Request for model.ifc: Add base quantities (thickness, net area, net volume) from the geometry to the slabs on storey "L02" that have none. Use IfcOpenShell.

First a look at what the model holds.

```python
import ifcopenshell
import ifcopenshell.util.element
import ifcopenshell.util.unit

model = ifcopenshell.open("model.ifc")
print(model.schema)
for unit_type in ("LENGTHUNIT", "AREAUNIT", "VOLUMEUNIT"):
    print(unit_type, ifcopenshell.util.unit.calculate_unit_scale(model, unit_type))
storey = next(s for s in model.by_type("IfcBuildingStorey") if s.Name == "L02")
slabs = [e for e in ifcopenshell.util.element.get_decomposition(storey) if e.is_a("IfcSlab")]
for e in sorted(slabs, key=lambda e: e.id()):
    print(e.id(), e.is_a(), e.Name, list(ifcopenshell.util.element.get_psets(e, qtos_only=True)), sep=" | ")
```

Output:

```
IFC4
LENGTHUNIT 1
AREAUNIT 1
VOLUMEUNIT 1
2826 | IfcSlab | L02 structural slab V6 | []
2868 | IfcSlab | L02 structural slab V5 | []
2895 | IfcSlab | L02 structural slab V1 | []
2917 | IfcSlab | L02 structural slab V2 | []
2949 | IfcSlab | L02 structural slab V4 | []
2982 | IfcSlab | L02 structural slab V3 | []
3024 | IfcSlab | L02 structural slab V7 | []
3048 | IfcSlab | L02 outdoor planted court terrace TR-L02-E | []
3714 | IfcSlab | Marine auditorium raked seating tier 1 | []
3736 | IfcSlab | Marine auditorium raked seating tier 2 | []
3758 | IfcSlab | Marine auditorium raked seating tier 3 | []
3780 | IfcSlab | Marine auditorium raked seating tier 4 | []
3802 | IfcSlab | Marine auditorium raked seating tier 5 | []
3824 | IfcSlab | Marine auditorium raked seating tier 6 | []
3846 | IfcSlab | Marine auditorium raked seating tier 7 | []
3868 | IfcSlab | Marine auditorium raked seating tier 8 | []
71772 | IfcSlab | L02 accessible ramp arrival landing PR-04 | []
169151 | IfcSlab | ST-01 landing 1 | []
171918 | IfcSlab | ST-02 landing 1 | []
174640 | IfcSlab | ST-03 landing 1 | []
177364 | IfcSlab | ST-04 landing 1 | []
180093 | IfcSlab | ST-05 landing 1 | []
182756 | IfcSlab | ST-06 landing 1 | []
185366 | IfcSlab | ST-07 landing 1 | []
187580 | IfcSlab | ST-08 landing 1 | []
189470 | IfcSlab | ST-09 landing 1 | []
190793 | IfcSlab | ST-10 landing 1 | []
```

```python
import ifcopenshell
import ifcopenshell.api.pset
import ifcopenshell.geom
import ifcopenshell.util.element
import ifcopenshell.util.shape
import ifcopenshell.util.unit

model = ifcopenshell.open("model.ifc")
unit_scale = ifcopenshell.util.unit.calculate_unit_scale(model)
area_scale = ifcopenshell.util.unit.calculate_unit_scale(model, "AREAUNIT")
volume_scale = ifcopenshell.util.unit.calculate_unit_scale(model, "VOLUMEUNIT")
settings = ifcopenshell.geom.settings()

storey = next(s for s in model.by_type("IfcBuildingStorey") if s.Name == "L02")
slabs = [e for e in ifcopenshell.util.element.get_decomposition(storey) if e.is_a("IfcSlab")]

for e in sorted(slabs, key=lambda e: e.id()):
    if ifcopenshell.util.element.get_psets(e, qtos_only=True, should_inherit=False):
        continue
    # Geometry comes back in metres, in the element's own axes.
    shape = ifcopenshell.geom.create_shape(settings, e)
    values = {
        "Width": ifcopenshell.util.shape.get_z(shape.geometry) / unit_scale,
        "NetArea": ifcopenshell.util.shape.get_footprint_area(shape.geometry) / area_scale,
        "NetVolume": ifcopenshell.util.shape.get_volume(shape.geometry) / volume_scale,
    }
    qto = ifcopenshell.api.pset.add_qto(model, product=e, name="Qto_SlabBaseQuantities")
    ifcopenshell.api.pset.edit_qto(model, qto=qto, properties=values)
    print(e.id(), {k: round(v, 3) for k, v in values.items()})

model.write("model_rev.ifc")
```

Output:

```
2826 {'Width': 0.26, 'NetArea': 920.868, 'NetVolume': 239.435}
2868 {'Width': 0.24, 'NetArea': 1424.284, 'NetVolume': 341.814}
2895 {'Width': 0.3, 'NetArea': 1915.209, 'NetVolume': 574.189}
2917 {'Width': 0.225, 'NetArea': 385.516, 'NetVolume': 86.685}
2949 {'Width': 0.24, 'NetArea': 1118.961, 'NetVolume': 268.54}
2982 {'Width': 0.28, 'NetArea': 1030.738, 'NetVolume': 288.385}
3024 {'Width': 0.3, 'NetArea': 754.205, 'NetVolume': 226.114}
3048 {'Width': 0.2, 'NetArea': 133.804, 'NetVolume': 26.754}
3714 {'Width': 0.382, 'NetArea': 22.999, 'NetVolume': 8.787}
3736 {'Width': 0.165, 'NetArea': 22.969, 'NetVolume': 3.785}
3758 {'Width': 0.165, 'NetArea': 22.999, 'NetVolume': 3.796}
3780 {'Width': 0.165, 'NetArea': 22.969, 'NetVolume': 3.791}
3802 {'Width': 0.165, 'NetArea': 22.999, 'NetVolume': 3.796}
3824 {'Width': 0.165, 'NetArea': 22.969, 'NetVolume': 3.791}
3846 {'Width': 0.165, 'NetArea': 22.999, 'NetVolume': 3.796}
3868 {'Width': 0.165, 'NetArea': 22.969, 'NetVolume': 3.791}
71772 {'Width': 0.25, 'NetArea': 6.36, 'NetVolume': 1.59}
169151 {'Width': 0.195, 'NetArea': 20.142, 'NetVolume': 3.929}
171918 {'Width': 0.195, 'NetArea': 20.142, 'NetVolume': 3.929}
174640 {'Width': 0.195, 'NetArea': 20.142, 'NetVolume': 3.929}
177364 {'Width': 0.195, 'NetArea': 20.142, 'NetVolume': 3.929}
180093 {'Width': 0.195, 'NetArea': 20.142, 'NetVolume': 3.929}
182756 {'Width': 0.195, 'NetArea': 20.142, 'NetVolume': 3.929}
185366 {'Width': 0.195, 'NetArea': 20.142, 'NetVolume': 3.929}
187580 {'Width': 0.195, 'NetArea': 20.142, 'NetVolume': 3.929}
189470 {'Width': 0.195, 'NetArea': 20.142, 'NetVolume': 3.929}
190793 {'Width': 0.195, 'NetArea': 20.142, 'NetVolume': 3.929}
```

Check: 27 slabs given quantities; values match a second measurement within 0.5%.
